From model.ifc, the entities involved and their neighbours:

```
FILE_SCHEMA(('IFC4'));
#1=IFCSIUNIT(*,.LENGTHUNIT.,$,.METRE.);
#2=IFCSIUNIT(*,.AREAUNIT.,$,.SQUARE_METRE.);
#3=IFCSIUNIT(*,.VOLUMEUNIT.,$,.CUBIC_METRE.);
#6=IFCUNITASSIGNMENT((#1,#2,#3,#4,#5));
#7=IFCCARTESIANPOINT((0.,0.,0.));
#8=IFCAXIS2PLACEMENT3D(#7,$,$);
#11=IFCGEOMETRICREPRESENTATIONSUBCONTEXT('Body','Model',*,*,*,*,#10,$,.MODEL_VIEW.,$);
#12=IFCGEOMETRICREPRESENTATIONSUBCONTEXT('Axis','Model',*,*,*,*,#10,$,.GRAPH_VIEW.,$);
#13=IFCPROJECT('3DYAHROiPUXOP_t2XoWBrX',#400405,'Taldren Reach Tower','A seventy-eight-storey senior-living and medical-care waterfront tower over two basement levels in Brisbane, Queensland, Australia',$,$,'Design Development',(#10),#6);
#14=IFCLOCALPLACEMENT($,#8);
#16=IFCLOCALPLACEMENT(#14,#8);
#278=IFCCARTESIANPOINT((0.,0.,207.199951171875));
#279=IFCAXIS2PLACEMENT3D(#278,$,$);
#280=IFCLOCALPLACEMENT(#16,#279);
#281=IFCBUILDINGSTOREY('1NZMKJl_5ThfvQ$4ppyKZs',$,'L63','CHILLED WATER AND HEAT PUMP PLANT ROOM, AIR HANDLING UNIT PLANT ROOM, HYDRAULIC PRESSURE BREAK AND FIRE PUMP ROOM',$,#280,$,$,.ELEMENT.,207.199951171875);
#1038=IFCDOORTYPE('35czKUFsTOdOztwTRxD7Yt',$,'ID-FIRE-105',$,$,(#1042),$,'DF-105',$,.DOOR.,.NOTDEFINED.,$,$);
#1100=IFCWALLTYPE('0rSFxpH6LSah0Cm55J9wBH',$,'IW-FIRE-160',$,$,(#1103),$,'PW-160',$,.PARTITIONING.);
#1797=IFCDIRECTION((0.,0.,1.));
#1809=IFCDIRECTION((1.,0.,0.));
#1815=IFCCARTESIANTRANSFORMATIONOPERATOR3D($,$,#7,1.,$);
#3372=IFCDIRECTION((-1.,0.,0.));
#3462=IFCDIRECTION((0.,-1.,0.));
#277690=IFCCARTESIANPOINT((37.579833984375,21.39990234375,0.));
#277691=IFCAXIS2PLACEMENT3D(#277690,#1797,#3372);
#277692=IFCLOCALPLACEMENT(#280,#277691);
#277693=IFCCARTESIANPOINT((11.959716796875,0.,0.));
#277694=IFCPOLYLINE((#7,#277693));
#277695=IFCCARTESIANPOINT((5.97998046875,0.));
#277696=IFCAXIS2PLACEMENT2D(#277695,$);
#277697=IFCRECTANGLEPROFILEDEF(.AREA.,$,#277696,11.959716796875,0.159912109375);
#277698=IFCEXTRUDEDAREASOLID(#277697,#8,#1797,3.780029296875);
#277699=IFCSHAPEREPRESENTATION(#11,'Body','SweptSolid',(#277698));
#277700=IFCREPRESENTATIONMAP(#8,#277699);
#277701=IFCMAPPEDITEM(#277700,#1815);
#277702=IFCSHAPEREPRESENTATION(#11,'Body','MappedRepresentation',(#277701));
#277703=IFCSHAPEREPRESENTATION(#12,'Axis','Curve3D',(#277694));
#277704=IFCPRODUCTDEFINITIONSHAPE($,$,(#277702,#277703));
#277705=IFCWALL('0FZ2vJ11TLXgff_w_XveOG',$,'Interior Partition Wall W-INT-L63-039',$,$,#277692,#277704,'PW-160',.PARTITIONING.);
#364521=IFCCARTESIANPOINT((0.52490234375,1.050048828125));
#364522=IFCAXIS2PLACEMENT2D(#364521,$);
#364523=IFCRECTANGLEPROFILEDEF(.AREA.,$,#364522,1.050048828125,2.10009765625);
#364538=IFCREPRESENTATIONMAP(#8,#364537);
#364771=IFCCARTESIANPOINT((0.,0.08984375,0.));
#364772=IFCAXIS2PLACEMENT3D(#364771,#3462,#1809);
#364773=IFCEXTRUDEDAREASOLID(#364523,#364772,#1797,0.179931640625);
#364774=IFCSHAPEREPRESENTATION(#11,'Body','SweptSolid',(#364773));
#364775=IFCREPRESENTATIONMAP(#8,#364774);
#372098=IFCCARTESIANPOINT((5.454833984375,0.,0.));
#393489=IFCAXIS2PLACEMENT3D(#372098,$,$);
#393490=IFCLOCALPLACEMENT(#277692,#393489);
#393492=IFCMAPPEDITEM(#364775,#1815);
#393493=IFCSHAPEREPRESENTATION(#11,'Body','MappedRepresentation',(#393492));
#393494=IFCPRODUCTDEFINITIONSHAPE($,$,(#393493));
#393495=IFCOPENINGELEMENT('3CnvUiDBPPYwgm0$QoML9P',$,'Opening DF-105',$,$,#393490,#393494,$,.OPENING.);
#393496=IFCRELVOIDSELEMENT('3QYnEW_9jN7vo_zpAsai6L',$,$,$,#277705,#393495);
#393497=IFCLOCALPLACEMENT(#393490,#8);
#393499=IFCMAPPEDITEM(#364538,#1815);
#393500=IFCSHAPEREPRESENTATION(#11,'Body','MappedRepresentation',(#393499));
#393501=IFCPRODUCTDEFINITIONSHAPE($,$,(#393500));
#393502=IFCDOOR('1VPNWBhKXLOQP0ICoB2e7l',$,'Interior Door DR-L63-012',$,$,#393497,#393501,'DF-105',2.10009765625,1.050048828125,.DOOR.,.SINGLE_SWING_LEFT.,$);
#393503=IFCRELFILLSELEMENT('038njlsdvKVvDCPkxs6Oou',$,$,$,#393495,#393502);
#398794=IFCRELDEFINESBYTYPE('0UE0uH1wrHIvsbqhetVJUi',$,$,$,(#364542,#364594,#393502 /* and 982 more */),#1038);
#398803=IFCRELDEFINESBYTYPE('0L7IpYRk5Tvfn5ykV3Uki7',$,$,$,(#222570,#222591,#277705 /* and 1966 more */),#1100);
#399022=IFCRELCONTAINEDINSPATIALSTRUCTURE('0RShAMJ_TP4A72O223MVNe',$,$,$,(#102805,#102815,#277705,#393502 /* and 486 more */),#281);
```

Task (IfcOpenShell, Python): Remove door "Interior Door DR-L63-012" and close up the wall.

```python
import ifcopenshell
import ifcopenshell.api.feature
import ifcopenshell.api.root
import ifcopenshell.geom
import ifcopenshell.util.shape

model = ifcopenshell.open("model.ifc")
settings = ifcopenshell.geom.settings()


def volume(element):
    """Net volume in cubic metres, openings subtracted."""
    shape = ifcopenshell.geom.create_shape(settings, element)
    return ifcopenshell.util.shape.get_volume(shape.geometry)


door = model.by_id(393502)
opening = door.FillsVoids[0].RelatingOpeningElement
wall = opening.VoidsElements[0].RelatingBuildingElement
before = volume(wall)

ifcopenshell.api.root.remove_product(model, product=door)
ifcopenshell.api.feature.remove_feature(model, feature=opening)

after = volume(wall)

print(f"wall volume {before:.3f} -> {after:.3f} m3")

model.write("model-out.ifc")
```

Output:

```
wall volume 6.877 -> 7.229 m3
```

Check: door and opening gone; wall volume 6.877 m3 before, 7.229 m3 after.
